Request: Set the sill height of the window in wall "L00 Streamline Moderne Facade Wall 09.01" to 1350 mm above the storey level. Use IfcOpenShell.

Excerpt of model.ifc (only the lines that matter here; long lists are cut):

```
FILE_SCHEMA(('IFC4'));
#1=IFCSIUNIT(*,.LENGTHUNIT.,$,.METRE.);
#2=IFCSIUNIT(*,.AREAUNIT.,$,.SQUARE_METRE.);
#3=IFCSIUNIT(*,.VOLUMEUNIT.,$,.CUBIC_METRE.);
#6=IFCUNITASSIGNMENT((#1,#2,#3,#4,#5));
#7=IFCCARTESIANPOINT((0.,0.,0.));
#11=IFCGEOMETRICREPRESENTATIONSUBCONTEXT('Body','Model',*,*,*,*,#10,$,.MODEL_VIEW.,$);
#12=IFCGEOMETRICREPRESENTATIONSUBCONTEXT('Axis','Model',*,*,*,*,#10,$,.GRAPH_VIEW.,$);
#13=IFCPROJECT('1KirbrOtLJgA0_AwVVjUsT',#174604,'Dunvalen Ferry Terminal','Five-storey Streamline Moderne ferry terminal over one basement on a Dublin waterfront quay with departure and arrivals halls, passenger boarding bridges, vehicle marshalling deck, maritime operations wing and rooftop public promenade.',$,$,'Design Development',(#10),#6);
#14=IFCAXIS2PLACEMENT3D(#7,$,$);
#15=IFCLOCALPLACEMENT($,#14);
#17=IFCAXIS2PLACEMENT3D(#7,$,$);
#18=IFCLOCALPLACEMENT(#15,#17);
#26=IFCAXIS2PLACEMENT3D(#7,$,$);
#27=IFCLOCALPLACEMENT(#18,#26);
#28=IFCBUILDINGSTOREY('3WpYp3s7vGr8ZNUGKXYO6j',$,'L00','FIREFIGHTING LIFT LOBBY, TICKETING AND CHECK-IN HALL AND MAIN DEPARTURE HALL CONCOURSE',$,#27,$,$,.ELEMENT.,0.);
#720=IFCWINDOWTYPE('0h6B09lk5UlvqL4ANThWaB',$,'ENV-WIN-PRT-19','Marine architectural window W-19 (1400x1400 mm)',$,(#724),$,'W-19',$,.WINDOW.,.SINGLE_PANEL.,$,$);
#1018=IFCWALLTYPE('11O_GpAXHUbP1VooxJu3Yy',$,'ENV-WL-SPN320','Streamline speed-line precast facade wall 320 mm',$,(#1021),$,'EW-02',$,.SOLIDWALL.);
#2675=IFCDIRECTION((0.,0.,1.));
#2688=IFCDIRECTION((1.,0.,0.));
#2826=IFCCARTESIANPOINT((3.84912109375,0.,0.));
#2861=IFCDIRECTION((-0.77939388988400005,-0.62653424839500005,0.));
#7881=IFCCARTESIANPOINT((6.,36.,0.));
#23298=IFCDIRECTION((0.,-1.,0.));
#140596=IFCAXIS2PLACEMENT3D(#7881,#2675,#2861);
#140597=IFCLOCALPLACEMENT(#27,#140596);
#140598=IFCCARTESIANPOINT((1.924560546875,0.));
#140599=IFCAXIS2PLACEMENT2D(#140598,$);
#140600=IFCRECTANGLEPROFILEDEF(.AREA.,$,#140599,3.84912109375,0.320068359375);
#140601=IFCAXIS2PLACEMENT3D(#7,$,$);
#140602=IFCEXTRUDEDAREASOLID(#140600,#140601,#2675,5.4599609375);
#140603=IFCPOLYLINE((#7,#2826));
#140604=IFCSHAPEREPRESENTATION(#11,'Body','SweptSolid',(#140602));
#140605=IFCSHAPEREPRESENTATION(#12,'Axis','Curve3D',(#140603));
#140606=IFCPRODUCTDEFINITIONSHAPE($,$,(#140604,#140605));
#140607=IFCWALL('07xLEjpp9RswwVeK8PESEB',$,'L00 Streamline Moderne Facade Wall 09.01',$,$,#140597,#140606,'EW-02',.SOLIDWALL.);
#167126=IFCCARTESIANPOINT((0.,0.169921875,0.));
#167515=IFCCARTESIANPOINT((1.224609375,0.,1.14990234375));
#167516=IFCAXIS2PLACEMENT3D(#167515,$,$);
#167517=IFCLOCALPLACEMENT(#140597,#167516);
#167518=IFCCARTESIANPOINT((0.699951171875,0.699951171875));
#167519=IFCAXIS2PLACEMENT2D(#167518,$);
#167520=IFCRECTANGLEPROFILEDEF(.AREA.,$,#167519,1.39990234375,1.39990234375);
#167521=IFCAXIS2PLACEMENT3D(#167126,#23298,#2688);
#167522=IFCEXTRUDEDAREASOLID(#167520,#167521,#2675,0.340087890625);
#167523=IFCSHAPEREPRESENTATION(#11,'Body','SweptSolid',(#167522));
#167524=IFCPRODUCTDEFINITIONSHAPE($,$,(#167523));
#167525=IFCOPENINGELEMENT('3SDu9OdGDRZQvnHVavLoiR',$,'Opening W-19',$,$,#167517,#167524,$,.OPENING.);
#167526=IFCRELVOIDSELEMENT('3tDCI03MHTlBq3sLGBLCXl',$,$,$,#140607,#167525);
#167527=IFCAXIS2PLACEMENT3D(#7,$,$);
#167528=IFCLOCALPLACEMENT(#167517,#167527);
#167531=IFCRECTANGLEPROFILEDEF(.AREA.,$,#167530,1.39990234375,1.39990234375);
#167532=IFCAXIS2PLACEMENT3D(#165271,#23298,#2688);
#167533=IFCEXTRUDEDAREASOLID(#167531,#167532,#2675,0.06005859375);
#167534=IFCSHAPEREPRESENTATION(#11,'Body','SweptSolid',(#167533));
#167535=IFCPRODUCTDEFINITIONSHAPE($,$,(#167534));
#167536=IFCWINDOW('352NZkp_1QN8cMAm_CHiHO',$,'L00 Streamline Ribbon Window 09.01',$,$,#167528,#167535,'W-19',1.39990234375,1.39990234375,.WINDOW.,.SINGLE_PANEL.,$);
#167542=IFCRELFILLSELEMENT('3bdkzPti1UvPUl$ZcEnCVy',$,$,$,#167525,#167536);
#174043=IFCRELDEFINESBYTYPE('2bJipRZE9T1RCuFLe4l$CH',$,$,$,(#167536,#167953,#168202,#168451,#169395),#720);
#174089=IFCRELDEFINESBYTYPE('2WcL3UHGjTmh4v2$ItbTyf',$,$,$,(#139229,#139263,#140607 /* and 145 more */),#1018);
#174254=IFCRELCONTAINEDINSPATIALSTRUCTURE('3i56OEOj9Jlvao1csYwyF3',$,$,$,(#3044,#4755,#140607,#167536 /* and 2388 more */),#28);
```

```python
import numpy as np
import ifcopenshell
import ifcopenshell.api.geometry
import ifcopenshell.geom
import ifcopenshell.util.element
import ifcopenshell.util.placement
import ifcopenshell.util.shape
import ifcopenshell.util.unit

model = ifcopenshell.open("model.ifc")
unit_scale = ifcopenshell.util.unit.calculate_unit_scale(model)

window = model.by_id(167536)
opening = window.FillsVoids[0].RelatingOpeningElement
storey = ifcopenshell.util.element.get_container(window, ifc_class="IfcBuildingStorey")
level = ifcopenshell.util.placement.get_local_placement(storey.ObjectPlacement)[2, 3]

# The opening's origin need not be at the sill, so measure its lowest point.
shape = ifcopenshell.geom.create_shape(ifcopenshell.geom.settings(), opening)
bottom = ifcopenshell.util.shape.get_shape_bottom_elevation(shape, shape.geometry) / unit_scale
dz = level + 1.35 / unit_scale - bottom

shift = np.array([0.0, 0.0, dz])
# The window is placed relative to its opening, so it follows when the opening moves.
matrix = ifcopenshell.util.placement.get_local_placement(opening.ObjectPlacement)
matrix[:3, 3] += shift
ifcopenshell.api.geometry.edit_object_placement(
    model, product=opening, matrix=matrix, is_si=False, should_transform_children=True
)

print(f"moved by {dz * unit_scale:+.3f} m")

model.write("model-out.ifc")
```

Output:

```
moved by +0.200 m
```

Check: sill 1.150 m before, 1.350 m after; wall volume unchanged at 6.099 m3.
